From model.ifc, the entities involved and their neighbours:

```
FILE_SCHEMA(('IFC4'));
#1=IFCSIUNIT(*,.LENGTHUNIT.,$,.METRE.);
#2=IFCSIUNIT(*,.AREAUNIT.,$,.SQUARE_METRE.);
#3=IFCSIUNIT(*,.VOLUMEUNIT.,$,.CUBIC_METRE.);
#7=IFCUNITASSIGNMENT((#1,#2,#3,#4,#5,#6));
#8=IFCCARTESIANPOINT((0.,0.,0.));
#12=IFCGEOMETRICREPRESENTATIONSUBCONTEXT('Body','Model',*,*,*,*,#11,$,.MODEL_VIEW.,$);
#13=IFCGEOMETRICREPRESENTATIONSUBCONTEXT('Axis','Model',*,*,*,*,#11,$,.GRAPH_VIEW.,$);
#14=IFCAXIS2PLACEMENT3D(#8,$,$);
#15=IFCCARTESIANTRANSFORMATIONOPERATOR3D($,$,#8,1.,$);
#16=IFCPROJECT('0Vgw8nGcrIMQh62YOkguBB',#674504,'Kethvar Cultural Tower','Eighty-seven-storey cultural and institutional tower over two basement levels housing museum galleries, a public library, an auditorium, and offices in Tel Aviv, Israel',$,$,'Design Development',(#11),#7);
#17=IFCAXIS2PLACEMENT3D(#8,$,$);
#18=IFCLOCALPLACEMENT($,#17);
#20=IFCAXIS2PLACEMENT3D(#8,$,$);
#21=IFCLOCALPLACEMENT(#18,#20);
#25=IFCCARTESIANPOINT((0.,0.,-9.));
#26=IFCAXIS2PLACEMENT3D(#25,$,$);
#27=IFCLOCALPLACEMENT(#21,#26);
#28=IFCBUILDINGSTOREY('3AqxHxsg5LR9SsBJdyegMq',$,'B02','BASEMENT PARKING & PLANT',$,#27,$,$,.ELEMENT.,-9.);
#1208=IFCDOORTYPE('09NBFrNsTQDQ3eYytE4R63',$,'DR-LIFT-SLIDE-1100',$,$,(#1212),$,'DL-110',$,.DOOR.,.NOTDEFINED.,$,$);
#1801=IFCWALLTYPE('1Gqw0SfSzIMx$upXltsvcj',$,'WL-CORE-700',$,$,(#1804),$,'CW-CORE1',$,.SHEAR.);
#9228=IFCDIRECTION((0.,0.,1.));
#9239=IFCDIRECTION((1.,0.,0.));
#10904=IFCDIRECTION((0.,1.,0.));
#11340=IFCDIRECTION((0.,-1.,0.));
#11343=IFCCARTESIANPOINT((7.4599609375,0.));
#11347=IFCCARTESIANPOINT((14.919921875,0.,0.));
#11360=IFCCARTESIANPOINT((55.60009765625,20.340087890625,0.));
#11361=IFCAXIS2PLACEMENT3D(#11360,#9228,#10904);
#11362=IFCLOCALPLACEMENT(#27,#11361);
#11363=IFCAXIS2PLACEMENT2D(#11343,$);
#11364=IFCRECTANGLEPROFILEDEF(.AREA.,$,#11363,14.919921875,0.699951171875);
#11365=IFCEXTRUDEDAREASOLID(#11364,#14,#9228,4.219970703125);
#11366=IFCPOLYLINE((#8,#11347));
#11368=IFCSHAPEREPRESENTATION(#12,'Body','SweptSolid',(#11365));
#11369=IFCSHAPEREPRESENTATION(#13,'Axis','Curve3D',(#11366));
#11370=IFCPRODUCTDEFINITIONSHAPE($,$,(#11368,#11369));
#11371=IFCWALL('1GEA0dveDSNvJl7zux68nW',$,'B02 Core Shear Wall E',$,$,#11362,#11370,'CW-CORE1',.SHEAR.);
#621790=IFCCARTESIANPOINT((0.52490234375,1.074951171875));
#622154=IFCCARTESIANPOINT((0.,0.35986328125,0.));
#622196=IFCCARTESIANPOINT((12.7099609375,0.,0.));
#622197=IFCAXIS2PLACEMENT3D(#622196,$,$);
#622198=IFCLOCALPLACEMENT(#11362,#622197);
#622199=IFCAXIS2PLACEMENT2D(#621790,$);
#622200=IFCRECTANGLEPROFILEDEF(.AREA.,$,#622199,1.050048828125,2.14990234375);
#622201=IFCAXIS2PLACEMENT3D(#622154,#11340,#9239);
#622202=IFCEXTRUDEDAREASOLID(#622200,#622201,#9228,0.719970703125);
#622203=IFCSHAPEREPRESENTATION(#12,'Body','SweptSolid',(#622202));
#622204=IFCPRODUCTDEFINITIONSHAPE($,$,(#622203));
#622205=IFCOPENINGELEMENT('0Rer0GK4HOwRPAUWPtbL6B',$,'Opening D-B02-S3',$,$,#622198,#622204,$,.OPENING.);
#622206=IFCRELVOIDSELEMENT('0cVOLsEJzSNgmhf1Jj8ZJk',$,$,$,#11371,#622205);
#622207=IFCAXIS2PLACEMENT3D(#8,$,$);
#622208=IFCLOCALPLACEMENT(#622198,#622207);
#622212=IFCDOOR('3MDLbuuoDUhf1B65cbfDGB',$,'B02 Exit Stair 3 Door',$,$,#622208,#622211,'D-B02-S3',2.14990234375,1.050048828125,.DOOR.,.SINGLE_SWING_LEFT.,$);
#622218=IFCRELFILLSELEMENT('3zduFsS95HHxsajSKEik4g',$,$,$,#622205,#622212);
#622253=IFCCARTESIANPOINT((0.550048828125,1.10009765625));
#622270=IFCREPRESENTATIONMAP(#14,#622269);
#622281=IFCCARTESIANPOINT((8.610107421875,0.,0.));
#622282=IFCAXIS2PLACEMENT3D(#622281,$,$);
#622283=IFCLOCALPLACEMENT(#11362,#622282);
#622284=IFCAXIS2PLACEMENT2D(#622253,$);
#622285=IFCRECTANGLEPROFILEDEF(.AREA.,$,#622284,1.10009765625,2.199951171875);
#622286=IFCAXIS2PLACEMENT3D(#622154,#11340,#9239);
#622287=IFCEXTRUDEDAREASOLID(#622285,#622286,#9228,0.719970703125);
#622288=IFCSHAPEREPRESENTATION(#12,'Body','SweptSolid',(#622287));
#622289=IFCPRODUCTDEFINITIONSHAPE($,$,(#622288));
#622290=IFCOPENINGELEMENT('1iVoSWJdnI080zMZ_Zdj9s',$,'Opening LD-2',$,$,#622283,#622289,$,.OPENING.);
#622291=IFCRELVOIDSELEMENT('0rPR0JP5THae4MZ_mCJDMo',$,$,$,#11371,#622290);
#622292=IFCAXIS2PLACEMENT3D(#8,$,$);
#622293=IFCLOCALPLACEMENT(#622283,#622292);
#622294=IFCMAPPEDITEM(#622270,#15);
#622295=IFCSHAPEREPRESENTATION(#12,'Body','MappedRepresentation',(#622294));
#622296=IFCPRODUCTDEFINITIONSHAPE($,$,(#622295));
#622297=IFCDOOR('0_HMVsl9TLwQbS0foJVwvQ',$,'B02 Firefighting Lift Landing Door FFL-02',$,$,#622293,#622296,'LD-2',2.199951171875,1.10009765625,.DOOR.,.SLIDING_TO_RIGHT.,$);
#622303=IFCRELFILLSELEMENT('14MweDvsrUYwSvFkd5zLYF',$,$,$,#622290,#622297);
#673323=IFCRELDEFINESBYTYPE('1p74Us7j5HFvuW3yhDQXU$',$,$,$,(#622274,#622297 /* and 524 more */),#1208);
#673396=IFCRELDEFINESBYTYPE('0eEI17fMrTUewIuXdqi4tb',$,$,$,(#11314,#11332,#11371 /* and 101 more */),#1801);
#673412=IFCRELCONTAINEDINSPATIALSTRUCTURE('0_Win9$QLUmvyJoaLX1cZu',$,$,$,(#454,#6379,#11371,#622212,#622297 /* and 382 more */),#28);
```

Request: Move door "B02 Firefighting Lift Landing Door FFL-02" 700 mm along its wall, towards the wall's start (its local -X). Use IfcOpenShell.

```python
import ifcopenshell
import ifcopenshell.api.geometry
import ifcopenshell.util.placement
import ifcopenshell.util.unit

model = ifcopenshell.open("model.ifc")
unit_scale = ifcopenshell.util.unit.calculate_unit_scale(model)

door = model.by_guid("0_HMVsl9TLwQbS0foJVwvQ")
opening = door.FillsVoids[0].RelatingOpeningElement
wall = opening.VoidsElements[0].RelatingBuildingElement

wall_matrix = ifcopenshell.util.placement.get_local_placement(wall.ObjectPlacement)
shift = wall_matrix[:3, 0] * -0.7 / unit_scale
before = ifcopenshell.util.placement.get_local_placement(door.ObjectPlacement)[:3, 3].copy()

# The door is placed relative to its opening, so it follows when the opening moves.
matrix = ifcopenshell.util.placement.get_local_placement(opening.ObjectPlacement)
matrix[:3, 3] += shift
ifcopenshell.api.geometry.edit_object_placement(
    model, product=opening, matrix=matrix, is_si=False, should_transform_children=True
)

after = ifcopenshell.util.placement.get_local_placement(door.ObjectPlacement)[:3, 3]
print("door moved by", (after - before).round(3) + 0.0)

model.write("model-out.ifc")
```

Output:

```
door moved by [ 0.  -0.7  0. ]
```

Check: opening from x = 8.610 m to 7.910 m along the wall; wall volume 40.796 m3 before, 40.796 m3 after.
